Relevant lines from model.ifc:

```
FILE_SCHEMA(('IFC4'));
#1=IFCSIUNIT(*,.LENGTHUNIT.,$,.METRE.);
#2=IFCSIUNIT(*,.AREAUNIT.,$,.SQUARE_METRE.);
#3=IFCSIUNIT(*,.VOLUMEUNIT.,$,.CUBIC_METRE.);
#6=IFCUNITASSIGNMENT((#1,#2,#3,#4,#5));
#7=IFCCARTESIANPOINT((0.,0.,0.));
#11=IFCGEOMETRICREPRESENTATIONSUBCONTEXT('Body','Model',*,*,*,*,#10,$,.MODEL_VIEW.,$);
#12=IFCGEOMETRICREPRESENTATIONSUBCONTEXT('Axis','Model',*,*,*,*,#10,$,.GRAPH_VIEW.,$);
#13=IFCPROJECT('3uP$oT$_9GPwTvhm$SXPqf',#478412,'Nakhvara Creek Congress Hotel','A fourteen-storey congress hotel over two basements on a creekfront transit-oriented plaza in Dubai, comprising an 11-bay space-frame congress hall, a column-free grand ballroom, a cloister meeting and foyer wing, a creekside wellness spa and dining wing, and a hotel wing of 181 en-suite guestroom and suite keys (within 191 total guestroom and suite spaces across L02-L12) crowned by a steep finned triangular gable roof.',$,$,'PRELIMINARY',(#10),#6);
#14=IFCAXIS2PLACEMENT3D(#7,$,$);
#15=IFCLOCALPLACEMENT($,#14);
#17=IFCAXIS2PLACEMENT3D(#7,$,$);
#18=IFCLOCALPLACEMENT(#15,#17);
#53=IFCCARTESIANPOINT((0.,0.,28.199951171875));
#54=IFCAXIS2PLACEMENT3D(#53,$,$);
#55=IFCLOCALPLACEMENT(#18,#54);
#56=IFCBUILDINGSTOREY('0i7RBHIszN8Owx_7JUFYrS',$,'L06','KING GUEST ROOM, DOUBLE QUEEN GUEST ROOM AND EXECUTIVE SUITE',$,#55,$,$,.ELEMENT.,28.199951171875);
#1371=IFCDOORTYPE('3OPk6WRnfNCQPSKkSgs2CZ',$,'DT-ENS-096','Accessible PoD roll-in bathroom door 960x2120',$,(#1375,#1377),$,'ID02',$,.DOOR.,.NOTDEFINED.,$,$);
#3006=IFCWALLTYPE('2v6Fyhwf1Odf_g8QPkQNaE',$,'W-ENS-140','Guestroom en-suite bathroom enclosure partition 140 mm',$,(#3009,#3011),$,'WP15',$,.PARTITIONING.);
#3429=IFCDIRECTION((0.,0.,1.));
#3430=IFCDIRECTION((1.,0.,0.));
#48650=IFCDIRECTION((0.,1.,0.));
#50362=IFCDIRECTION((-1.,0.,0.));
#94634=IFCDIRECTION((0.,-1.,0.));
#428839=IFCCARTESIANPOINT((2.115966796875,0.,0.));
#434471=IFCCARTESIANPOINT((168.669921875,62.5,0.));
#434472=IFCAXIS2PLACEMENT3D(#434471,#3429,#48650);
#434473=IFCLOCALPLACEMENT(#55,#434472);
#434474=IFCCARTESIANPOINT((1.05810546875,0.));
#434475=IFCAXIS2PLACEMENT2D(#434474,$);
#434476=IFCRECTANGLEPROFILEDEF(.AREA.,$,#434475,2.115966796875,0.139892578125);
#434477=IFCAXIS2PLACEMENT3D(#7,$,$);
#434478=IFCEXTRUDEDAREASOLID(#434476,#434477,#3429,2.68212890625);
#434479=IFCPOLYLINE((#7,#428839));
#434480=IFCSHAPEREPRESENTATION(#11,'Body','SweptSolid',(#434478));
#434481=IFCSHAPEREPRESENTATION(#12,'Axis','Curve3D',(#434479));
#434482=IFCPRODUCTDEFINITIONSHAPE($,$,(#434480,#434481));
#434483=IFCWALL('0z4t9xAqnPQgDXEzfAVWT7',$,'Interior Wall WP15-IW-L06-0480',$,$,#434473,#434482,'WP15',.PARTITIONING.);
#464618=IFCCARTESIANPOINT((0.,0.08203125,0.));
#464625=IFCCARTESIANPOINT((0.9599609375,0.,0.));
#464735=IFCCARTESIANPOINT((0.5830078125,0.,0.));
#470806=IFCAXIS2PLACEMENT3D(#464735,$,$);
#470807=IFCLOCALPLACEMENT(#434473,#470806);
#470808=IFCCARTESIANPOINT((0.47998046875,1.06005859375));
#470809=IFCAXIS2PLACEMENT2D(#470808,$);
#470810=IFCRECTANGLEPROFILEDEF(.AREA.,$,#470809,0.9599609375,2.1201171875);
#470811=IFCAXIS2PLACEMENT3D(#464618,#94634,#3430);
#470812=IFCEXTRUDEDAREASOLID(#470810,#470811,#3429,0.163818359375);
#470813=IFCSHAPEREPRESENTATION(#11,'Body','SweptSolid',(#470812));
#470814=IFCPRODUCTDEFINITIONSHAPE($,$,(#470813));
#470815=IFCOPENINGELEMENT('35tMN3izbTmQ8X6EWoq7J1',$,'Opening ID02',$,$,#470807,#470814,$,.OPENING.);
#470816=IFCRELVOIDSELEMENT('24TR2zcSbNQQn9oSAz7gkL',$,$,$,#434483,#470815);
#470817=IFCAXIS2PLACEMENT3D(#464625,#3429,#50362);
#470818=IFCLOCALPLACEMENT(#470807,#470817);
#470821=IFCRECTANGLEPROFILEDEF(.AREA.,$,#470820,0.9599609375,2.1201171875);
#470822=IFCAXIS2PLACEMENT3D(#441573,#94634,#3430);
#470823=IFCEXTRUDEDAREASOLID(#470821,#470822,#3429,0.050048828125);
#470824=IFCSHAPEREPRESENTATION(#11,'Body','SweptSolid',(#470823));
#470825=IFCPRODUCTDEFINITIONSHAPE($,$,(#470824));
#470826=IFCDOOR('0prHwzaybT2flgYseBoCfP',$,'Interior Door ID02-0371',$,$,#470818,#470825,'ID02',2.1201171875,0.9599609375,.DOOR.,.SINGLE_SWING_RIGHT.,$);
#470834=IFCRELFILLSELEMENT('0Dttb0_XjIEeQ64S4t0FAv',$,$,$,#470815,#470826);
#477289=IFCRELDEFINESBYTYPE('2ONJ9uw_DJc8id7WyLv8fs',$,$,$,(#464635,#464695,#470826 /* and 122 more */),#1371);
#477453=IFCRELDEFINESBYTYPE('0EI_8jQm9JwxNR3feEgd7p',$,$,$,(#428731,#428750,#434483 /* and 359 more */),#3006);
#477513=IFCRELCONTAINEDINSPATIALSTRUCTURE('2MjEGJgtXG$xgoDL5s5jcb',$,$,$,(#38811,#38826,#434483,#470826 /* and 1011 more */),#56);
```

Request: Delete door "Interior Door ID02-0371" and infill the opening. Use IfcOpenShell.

```python
import ifcopenshell
import ifcopenshell.api.feature
import ifcopenshell.api.root
import ifcopenshell.geom
import ifcopenshell.util.shape

model = ifcopenshell.open("model.ifc")
settings = ifcopenshell.geom.settings()


def volume(element):
    """Net volume in cubic metres, openings subtracted."""
    shape = ifcopenshell.geom.create_shape(settings, element)
    return ifcopenshell.util.shape.get_volume(shape.geometry)


door = model.by_id(470826)
opening = door.FillsVoids[0].RelatingOpeningElement
wall = opening.VoidsElements[0].RelatingBuildingElement
before = volume(wall)

ifcopenshell.api.root.remove_product(model, product=door)
ifcopenshell.api.feature.remove_feature(model, feature=opening)

after = volume(wall)

print(f"wall volume {before:.3f} -> {after:.3f} m3")

model.write("model-out.ifc")
```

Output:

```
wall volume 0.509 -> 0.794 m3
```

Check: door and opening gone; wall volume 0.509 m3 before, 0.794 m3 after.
